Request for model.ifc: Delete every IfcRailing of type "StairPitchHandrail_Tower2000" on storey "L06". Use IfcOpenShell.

First a look at what the model holds.

```python
import ifcopenshell
import ifcopenshell.util.element

model = ifcopenshell.open("model.ifc")
print(model.schema)
storey = next(s for s in model.by_type("IfcBuildingStorey") if s.Name == "L06")
railings = [e for e in ifcopenshell.util.element.get_decomposition(storey) if e.is_a("IfcRailing")]
seen = {}
for e in railings:
    element_type = ifcopenshell.util.element.get_type(e)
    name = element_type.Name if element_type not in (None, e) else None
    seen[name] = seen.get(name, 0) + 1
for name, count in sorted(seen.items(), key=str):
    print(count, "x", name)
```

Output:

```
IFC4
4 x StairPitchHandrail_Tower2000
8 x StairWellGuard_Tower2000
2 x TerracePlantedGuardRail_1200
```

```python
import ifcopenshell
import ifcopenshell.api.root
import ifcopenshell.util.element

model = ifcopenshell.open("model.ifc")

storey = next(s for s in model.by_type("IfcBuildingStorey") if s.Name == "L06")
railings = [e for e in ifcopenshell.util.element.get_decomposition(storey) if e.is_a("IfcRailing")]
targets = [e for e in railings if (t := ifcopenshell.util.element.get_type(e)) not in (None, e) and t.Name == "StairPitchHandrail_Tower2000"]

for e in targets:
    ifcopenshell.api.root.remove_product(model, product=e)
print(len(targets), "removed")

model.write("model-out.ifc")
```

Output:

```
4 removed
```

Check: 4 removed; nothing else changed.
